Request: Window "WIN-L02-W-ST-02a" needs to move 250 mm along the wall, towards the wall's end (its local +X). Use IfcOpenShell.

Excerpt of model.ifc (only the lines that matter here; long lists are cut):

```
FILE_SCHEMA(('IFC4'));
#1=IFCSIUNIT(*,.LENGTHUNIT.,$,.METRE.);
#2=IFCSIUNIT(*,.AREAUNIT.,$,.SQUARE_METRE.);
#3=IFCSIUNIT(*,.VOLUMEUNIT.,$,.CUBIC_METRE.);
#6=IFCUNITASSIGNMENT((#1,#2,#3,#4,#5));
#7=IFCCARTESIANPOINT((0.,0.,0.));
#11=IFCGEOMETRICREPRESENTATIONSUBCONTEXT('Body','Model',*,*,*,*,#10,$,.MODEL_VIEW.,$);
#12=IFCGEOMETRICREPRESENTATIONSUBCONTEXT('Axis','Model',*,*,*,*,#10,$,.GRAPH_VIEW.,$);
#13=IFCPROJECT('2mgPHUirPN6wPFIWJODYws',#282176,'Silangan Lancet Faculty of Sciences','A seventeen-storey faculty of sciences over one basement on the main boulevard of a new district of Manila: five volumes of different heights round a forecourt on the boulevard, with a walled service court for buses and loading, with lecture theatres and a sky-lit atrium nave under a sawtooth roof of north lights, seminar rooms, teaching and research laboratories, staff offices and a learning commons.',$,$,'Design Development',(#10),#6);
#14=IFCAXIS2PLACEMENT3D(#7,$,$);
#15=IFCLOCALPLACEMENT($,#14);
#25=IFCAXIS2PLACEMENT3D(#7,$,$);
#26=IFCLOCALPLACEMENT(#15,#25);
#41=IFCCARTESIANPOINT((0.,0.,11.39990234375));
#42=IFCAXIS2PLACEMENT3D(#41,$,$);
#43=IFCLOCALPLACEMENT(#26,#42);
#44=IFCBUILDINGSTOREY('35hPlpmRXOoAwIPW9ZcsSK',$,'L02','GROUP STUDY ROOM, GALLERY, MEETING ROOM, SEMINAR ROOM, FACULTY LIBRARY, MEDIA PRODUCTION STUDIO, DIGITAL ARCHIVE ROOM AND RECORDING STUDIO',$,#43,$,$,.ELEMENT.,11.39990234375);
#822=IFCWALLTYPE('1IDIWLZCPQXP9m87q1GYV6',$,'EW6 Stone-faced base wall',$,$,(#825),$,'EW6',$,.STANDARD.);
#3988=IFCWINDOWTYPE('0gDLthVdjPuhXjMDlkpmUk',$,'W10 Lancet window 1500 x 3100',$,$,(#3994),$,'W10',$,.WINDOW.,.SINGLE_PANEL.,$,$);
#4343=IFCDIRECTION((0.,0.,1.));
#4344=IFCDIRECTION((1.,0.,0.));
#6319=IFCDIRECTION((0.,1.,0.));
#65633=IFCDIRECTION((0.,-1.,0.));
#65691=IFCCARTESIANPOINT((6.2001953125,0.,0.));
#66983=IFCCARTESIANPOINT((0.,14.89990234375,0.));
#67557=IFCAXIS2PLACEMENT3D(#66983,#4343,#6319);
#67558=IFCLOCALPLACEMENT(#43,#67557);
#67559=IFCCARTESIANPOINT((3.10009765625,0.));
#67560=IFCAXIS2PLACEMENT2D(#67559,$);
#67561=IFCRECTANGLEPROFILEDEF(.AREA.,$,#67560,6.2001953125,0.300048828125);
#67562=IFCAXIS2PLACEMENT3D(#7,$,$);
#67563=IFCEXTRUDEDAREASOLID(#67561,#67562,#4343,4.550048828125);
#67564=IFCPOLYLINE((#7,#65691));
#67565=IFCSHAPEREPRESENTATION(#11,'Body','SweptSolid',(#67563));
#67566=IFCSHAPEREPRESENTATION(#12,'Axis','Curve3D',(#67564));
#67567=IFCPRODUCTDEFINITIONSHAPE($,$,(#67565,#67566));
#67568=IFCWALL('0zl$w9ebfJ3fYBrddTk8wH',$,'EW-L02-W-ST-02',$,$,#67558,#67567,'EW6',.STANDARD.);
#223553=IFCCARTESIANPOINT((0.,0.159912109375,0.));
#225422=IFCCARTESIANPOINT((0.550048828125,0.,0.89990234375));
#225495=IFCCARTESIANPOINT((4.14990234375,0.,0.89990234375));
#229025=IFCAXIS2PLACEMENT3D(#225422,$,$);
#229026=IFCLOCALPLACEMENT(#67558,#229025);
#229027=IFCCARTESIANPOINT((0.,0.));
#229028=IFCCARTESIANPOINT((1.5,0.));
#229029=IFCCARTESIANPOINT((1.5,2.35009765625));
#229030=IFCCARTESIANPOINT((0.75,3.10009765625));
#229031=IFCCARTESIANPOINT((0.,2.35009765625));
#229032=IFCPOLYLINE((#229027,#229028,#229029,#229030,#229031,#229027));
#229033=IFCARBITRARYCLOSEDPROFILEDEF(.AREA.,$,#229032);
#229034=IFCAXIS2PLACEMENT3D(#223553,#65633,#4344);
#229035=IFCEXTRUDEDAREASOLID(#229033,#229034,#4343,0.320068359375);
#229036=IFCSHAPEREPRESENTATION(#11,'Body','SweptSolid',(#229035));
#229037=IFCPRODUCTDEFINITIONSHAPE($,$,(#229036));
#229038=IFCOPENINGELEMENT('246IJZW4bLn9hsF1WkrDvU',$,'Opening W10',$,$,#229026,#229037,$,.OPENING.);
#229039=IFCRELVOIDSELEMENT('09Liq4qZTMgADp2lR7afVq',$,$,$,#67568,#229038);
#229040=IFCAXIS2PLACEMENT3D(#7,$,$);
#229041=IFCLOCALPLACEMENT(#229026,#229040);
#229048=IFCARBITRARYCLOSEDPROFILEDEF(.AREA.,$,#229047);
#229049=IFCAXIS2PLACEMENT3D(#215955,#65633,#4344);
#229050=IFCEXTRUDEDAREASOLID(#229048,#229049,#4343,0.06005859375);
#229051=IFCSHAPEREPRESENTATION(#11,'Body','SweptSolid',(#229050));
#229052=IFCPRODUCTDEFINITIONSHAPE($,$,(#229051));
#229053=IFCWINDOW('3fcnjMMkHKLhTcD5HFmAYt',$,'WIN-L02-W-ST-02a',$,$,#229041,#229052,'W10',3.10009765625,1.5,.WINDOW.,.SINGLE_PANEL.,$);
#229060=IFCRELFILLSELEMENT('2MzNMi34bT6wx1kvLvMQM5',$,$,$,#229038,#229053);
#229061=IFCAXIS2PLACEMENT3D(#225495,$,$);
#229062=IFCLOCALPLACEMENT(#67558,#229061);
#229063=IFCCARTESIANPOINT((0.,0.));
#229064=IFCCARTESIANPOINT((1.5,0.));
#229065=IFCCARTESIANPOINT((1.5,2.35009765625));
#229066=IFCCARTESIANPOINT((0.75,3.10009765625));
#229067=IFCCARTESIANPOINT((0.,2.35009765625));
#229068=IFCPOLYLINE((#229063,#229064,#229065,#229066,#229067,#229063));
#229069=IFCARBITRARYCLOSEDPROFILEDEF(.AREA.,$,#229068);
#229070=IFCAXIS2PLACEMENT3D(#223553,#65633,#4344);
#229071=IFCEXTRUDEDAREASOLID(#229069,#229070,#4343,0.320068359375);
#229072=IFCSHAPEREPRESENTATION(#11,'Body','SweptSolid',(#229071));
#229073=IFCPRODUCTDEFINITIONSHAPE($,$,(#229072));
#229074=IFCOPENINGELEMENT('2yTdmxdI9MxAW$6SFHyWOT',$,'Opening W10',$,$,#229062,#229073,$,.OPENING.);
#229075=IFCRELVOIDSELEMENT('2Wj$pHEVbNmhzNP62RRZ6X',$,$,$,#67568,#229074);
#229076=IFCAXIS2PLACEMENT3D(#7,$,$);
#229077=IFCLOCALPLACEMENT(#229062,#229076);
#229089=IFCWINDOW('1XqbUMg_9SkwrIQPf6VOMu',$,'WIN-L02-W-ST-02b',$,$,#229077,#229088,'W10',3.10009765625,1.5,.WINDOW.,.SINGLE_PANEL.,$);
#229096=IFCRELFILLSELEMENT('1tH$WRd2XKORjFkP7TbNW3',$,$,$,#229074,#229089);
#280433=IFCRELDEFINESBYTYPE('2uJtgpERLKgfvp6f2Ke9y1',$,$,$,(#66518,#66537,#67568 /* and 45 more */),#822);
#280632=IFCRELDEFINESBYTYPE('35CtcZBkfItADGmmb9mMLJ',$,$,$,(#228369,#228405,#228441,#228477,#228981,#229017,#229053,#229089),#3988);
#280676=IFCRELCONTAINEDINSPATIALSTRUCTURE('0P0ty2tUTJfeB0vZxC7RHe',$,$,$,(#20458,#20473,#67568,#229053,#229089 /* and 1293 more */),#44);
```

```python
import ifcopenshell
import ifcopenshell.api.geometry
import ifcopenshell.util.placement
import ifcopenshell.util.unit

model = ifcopenshell.open("model.ifc")
unit_scale = ifcopenshell.util.unit.calculate_unit_scale(model)

window = model.by_guid("3fcnjMMkHKLhTcD5HFmAYt")
opening = window.FillsVoids[0].RelatingOpeningElement
wall = opening.VoidsElements[0].RelatingBuildingElement

wall_matrix = ifcopenshell.util.placement.get_local_placement(wall.ObjectPlacement)
shift = wall_matrix[:3, 0] * 0.25 / unit_scale
before = ifcopenshell.util.placement.get_local_placement(window.ObjectPlacement)[:3, 3].copy()

# The window is placed relative to its opening, so it follows when the opening moves.
matrix = ifcopenshell.util.placement.get_local_placement(opening.ObjectPlacement)
matrix[:3, 3] += shift
ifcopenshell.api.geometry.edit_object_placement(
    model, product=opening, matrix=matrix, is_si=False, should_transform_children=True
)

after = ifcopenshell.util.placement.get_local_placement(window.ObjectPlacement)[:3, 3]
print("window moved by", (after - before).round(3) + 0.0)

model.write("model_v2.ifc")
```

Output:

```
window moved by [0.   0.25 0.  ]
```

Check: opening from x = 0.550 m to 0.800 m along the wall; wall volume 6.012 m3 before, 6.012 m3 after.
